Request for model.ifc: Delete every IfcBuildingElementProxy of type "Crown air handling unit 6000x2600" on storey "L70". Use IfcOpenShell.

First a look at what the model holds.

```python
import ifcopenshell
import ifcopenshell.util.element

model = ifcopenshell.open("model.ifc")
print(model.schema)
storey = next(s for s in model.by_type("IfcBuildingStorey") if s.Name == "L70")
proxies = [e for e in ifcopenshell.util.element.get_decomposition(storey) if e.is_a("IfcBuildingElementProxy")]
seen = {}
for e in proxies:
    element_type = ifcopenshell.util.element.get_type(e)
    name = element_type.Name if element_type not in (None, e) else None
    seen[name] = seen.get(name, 0) + 1
for name, count in sorted(seen.items(), key=str):
    print(count, "x", name)
```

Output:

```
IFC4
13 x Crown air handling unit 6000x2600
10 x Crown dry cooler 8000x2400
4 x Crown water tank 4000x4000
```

```python
import ifcopenshell
import ifcopenshell.api.root
import ifcopenshell.util.element

model = ifcopenshell.open("model.ifc")

storey = next(s for s in model.by_type("IfcBuildingStorey") if s.Name == "L70")
proxies = [e for e in ifcopenshell.util.element.get_decomposition(storey) if e.is_a("IfcBuildingElementProxy")]
targets = [e for e in proxies if (t := ifcopenshell.util.element.get_type(e)) not in (None, e) and t.Name == "Crown air handling unit 6000x2600"]

for e in targets:
    ifcopenshell.api.root.remove_product(model, product=e)
print(len(targets), "removed")

model.write("model_edited.ifc")
```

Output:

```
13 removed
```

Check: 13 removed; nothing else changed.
